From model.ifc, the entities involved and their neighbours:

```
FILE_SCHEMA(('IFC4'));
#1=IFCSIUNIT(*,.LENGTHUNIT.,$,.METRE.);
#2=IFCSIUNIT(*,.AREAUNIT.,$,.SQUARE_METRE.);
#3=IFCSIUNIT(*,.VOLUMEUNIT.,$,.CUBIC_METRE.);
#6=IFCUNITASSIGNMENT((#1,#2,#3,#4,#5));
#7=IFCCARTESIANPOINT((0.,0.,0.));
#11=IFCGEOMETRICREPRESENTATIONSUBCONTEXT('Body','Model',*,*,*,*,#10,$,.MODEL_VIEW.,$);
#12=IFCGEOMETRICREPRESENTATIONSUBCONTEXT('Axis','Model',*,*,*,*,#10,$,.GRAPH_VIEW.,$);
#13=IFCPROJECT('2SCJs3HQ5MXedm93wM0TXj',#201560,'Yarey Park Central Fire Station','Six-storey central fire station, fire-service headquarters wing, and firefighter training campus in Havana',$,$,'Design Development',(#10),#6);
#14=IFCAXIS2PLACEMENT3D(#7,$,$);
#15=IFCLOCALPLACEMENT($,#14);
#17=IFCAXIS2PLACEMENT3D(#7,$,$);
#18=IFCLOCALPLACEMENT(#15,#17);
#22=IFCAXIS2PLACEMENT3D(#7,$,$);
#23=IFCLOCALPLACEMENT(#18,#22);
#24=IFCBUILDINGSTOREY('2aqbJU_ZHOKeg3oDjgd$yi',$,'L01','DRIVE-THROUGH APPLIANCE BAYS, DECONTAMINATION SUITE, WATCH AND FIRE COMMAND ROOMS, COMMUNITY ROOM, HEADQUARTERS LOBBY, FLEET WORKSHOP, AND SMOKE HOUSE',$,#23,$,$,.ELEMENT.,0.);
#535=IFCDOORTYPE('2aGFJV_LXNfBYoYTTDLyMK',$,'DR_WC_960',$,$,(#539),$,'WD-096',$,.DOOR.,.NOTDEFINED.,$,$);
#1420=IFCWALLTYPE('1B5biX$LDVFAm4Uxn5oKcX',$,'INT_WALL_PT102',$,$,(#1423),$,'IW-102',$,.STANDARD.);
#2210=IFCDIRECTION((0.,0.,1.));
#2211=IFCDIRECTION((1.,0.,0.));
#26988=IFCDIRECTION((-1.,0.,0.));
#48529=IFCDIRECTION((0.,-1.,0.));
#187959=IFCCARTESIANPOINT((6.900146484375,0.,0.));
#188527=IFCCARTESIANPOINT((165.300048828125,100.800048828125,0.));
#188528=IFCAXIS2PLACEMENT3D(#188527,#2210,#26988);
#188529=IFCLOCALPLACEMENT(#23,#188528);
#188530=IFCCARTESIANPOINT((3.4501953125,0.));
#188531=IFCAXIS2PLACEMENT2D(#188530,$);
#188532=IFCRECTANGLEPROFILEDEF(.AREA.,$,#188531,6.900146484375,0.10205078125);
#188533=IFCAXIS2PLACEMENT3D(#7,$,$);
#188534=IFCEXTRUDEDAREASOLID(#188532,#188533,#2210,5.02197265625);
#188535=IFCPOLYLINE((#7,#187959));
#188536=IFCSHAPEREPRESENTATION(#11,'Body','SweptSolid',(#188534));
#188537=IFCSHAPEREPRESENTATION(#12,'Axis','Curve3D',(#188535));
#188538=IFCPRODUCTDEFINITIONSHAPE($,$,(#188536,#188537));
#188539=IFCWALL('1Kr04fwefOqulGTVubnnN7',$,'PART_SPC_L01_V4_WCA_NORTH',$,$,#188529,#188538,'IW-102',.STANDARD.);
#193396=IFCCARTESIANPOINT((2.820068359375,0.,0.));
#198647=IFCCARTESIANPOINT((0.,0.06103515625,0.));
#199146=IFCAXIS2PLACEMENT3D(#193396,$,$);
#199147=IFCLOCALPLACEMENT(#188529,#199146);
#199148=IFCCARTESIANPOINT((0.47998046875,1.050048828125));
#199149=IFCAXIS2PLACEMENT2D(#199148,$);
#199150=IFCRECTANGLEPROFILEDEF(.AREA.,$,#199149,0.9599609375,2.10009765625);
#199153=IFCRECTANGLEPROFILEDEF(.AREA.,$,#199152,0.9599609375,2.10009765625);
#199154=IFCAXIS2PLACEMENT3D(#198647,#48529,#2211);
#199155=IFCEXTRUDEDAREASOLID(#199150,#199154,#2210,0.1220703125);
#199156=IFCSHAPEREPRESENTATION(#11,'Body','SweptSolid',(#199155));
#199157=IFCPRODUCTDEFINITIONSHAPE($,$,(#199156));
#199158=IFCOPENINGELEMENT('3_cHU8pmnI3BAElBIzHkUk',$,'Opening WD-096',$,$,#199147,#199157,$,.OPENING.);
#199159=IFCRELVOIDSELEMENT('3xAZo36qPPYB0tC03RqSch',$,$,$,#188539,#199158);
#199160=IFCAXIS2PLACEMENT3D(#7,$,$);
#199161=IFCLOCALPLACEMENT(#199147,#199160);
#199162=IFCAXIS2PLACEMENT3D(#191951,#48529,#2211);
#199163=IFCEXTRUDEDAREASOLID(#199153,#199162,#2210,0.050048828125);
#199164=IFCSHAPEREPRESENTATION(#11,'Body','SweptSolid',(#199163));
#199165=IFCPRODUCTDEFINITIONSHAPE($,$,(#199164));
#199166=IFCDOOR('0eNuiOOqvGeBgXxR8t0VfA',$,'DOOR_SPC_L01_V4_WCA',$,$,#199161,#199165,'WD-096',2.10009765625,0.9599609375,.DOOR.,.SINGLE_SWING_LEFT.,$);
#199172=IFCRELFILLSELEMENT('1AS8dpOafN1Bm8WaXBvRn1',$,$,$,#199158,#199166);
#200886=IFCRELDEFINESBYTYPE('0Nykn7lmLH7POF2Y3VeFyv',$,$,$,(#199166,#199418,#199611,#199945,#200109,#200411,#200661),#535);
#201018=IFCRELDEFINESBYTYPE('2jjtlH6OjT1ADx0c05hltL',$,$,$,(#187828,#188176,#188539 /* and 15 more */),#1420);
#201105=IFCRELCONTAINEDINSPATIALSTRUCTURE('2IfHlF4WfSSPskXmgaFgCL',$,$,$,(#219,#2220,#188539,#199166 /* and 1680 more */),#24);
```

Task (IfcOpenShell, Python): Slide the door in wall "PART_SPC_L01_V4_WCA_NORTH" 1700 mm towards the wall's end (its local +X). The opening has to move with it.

```python
import ifcopenshell
import ifcopenshell.api.geometry
import ifcopenshell.util.placement

model = ifcopenshell.open("model.ifc")

door = model.by_id(199166)
opening = door.FillsVoids[0].RelatingOpeningElement
wall = opening.VoidsElements[0].RelatingBuildingElement

wall_matrix = ifcopenshell.util.placement.get_local_placement(wall.ObjectPlacement)
shift = wall_matrix[:3, 0] * 1.7
before = ifcopenshell.util.placement.get_local_placement(door.ObjectPlacement)[:3, 3].copy()

# The door is placed relative to its opening, so it follows when the opening moves.
matrix = ifcopenshell.util.placement.get_local_placement(opening.ObjectPlacement)
matrix[:3, 3] += shift
ifcopenshell.api.geometry.edit_object_placement(
    model, product=opening, matrix=matrix, is_si=False, should_transform_children=True
)

after = ifcopenshell.util.placement.get_local_placement(door.ObjectPlacement)[:3, 3]
print("door moved by", (after - before).round(3) + 0.0)

model.write("model-out.ifc")
```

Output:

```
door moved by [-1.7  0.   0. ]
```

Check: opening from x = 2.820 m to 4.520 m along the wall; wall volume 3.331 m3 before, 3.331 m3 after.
